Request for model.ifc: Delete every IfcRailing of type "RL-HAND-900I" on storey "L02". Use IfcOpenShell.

First a look at what the model holds.

```python
import ifcopenshell
import ifcopenshell.util.element

model = ifcopenshell.open("model.ifc")
print(model.schema)
storey = next(s for s in model.by_type("IfcBuildingStorey") if s.Name == "L02")
railings = [e for e in ifcopenshell.util.element.get_decomposition(storey) if e.is_a("IfcRailing")]
seen = {}
for e in railings:
    element_type = ifcopenshell.util.element.get_type(e)
    name = element_type.Name if element_type not in (None, e) else None
    seen[name] = seen.get(name, 0) + 1
for name, count in sorted(seen.items(), key=str):
    print(count, "x", name)
```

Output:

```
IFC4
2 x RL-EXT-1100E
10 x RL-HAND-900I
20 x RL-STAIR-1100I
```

```python
import ifcopenshell
import ifcopenshell.api.root
import ifcopenshell.util.element

model = ifcopenshell.open("model.ifc")

storey = next(s for s in model.by_type("IfcBuildingStorey") if s.Name == "L02")
railings = [e for e in ifcopenshell.util.element.get_decomposition(storey) if e.is_a("IfcRailing")]
targets = [e for e in railings if (t := ifcopenshell.util.element.get_type(e)) not in (None, e) and t.Name == "RL-HAND-900I"]

for e in targets:
    ifcopenshell.api.root.remove_product(model, product=e)
print(len(targets), "removed")

model.write("model_v2.ifc")
```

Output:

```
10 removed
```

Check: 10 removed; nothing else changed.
